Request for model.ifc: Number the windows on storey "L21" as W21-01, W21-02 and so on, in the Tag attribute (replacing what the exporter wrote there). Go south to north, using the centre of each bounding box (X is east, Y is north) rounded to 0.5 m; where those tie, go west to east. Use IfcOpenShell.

First a look at what the model holds.

```python
import ifcopenshell
import ifcopenshell.util.element
import ifcopenshell.util.placement

model = ifcopenshell.open("model.ifc")
print(model.schema)
storey = next(s for s in model.by_type("IfcBuildingStorey") if s.Name == "L21")
windows = [e for e in ifcopenshell.util.element.get_decomposition(storey) if e.is_a("IfcWindow")]
for e in sorted(windows, key=lambda e: e.id()):
    origin = ifcopenshell.util.placement.get_local_placement(e.ObjectPlacement)[:3, 3]
    print(e.id(), e.Tag, e.Name, origin.round(2) + 0.0, sep=" | ")
```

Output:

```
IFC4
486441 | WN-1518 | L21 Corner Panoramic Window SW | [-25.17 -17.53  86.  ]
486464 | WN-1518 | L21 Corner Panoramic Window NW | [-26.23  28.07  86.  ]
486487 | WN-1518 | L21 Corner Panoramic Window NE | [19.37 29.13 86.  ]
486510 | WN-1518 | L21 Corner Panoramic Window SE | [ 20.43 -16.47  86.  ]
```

```python
import ifcopenshell
import ifcopenshell.geom
import ifcopenshell.util.element
import ifcopenshell.util.shape

model = ifcopenshell.open("model.ifc")
settings = ifcopenshell.geom.settings()
settings.set("use-world-coords", True)


def centre(element):
    shape = ifcopenshell.geom.create_shape(settings, element)
    return ifcopenshell.util.shape.get_bbox_centroid(shape.geometry)


storey = next(s for s in model.by_type("IfcBuildingStorey") if s.Name == "L21")
windows = [e for e in ifcopenshell.util.element.get_decomposition(storey) if e.is_a("IfcWindow")]

# Insertion points can sit at a corner or the storey origin, so sort by the geometry (in metres).
centres = {e: centre(e) for e in windows}
windows.sort(key=lambda e: (round(centres[e][1] / 0.5), centres[e][0]))

for i, e in enumerate(windows, start=1):
    number = f"W21-{i:02d}"
    e.Tag = number
    print(e.id(), number)

model.write("model-out.ifc")
```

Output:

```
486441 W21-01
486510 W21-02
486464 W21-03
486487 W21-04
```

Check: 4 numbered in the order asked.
